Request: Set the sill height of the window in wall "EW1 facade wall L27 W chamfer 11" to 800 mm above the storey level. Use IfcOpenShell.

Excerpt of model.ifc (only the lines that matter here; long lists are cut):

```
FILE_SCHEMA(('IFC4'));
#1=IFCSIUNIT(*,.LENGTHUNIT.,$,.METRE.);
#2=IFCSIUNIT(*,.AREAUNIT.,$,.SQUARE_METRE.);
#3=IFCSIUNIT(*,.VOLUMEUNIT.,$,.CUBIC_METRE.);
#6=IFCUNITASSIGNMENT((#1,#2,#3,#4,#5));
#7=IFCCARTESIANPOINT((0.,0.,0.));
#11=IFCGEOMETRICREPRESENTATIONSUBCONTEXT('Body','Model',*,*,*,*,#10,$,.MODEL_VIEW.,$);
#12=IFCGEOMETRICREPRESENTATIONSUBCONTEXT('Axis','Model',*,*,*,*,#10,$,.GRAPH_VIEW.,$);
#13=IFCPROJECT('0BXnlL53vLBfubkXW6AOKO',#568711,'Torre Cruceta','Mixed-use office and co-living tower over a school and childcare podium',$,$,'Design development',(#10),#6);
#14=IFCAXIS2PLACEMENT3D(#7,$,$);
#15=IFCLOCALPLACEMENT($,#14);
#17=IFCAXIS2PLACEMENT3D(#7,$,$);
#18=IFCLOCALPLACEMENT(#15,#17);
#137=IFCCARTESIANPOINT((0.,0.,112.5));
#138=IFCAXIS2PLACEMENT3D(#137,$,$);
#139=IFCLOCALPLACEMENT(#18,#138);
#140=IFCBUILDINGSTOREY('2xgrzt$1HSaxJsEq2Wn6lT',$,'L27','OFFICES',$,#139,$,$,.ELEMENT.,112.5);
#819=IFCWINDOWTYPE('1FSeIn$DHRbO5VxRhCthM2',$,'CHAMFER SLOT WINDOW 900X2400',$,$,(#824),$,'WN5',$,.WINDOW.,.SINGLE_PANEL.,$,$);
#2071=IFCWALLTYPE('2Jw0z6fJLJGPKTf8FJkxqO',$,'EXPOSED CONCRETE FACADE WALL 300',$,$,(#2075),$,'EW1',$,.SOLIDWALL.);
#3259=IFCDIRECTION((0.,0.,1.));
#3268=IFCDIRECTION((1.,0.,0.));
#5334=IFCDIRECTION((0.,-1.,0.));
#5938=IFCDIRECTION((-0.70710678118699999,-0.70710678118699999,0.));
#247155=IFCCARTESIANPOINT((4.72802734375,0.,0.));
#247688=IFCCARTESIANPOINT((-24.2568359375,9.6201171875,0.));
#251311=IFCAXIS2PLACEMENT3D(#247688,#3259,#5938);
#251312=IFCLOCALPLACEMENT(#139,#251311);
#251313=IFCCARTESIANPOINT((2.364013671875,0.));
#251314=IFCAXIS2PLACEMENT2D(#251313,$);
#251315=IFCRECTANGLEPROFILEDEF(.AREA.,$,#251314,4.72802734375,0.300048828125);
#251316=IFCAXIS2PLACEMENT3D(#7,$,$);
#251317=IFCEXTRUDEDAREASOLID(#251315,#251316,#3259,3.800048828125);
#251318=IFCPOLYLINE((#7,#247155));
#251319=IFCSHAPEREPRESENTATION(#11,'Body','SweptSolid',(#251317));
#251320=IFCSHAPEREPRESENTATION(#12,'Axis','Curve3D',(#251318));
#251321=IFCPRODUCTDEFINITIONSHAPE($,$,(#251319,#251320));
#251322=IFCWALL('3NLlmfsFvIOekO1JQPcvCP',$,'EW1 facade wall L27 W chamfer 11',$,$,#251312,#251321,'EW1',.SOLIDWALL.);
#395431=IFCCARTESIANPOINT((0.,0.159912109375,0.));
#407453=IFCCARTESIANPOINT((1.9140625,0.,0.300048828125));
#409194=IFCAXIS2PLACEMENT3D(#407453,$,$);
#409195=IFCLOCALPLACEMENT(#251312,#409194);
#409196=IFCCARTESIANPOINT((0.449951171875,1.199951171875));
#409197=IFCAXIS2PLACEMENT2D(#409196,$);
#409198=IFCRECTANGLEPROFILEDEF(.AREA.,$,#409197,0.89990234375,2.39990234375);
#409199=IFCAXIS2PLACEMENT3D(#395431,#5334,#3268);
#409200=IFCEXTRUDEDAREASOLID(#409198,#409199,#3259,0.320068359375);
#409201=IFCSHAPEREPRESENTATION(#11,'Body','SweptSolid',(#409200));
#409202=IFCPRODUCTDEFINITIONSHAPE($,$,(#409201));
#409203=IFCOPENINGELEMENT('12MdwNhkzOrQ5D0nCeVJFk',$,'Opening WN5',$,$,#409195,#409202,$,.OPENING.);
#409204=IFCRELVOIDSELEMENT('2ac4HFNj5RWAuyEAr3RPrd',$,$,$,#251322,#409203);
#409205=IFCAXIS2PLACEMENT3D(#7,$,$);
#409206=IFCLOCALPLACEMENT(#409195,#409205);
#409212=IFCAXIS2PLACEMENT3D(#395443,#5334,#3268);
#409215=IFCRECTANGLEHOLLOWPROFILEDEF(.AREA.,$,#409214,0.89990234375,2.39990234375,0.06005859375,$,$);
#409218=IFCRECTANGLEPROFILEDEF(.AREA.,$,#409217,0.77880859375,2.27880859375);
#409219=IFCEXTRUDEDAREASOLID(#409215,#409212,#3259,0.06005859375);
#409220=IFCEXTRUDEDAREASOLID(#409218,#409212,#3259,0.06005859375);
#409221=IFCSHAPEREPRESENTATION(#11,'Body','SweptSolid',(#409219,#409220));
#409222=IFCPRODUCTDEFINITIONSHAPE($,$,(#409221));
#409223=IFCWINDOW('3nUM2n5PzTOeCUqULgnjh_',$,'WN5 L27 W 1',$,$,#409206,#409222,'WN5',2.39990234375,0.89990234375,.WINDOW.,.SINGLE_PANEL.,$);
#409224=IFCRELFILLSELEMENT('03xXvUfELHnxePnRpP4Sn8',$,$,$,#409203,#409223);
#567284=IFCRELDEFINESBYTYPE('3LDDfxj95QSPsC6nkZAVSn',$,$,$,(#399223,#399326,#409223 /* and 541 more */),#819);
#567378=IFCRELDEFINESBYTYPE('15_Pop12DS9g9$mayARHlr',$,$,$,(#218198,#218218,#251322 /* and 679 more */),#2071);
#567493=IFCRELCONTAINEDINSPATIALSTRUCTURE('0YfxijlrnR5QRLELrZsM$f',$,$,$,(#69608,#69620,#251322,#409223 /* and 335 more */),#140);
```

```python
import numpy as np
import ifcopenshell
import ifcopenshell.api.geometry
import ifcopenshell.geom
import ifcopenshell.util.element
import ifcopenshell.util.placement
import ifcopenshell.util.shape
import ifcopenshell.util.unit

model = ifcopenshell.open("model.ifc")
unit_scale = ifcopenshell.util.unit.calculate_unit_scale(model)

window = model.by_id(409223)
opening = window.FillsVoids[0].RelatingOpeningElement
storey = ifcopenshell.util.element.get_container(window, ifc_class="IfcBuildingStorey")
level = ifcopenshell.util.placement.get_local_placement(storey.ObjectPlacement)[2, 3]

# The opening's origin need not be at the sill, so measure its lowest point.
shape = ifcopenshell.geom.create_shape(ifcopenshell.geom.settings(), opening)
bottom = ifcopenshell.util.shape.get_shape_bottom_elevation(shape, shape.geometry) / unit_scale
dz = level + 0.8 / unit_scale - bottom

shift = np.array([0.0, 0.0, dz])
# The window is placed relative to its opening, so it follows when the opening moves.
matrix = ifcopenshell.util.placement.get_local_placement(opening.ObjectPlacement)
matrix[:3, 3] += shift
ifcopenshell.api.geometry.edit_object_placement(
    model, product=opening, matrix=matrix, is_si=False, should_transform_children=True
)

print(f"moved by {dz * unit_scale:+.3f} m")

model.write("model_updated.ifc")
```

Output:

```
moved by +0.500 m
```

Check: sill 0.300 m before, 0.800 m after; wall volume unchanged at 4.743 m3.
